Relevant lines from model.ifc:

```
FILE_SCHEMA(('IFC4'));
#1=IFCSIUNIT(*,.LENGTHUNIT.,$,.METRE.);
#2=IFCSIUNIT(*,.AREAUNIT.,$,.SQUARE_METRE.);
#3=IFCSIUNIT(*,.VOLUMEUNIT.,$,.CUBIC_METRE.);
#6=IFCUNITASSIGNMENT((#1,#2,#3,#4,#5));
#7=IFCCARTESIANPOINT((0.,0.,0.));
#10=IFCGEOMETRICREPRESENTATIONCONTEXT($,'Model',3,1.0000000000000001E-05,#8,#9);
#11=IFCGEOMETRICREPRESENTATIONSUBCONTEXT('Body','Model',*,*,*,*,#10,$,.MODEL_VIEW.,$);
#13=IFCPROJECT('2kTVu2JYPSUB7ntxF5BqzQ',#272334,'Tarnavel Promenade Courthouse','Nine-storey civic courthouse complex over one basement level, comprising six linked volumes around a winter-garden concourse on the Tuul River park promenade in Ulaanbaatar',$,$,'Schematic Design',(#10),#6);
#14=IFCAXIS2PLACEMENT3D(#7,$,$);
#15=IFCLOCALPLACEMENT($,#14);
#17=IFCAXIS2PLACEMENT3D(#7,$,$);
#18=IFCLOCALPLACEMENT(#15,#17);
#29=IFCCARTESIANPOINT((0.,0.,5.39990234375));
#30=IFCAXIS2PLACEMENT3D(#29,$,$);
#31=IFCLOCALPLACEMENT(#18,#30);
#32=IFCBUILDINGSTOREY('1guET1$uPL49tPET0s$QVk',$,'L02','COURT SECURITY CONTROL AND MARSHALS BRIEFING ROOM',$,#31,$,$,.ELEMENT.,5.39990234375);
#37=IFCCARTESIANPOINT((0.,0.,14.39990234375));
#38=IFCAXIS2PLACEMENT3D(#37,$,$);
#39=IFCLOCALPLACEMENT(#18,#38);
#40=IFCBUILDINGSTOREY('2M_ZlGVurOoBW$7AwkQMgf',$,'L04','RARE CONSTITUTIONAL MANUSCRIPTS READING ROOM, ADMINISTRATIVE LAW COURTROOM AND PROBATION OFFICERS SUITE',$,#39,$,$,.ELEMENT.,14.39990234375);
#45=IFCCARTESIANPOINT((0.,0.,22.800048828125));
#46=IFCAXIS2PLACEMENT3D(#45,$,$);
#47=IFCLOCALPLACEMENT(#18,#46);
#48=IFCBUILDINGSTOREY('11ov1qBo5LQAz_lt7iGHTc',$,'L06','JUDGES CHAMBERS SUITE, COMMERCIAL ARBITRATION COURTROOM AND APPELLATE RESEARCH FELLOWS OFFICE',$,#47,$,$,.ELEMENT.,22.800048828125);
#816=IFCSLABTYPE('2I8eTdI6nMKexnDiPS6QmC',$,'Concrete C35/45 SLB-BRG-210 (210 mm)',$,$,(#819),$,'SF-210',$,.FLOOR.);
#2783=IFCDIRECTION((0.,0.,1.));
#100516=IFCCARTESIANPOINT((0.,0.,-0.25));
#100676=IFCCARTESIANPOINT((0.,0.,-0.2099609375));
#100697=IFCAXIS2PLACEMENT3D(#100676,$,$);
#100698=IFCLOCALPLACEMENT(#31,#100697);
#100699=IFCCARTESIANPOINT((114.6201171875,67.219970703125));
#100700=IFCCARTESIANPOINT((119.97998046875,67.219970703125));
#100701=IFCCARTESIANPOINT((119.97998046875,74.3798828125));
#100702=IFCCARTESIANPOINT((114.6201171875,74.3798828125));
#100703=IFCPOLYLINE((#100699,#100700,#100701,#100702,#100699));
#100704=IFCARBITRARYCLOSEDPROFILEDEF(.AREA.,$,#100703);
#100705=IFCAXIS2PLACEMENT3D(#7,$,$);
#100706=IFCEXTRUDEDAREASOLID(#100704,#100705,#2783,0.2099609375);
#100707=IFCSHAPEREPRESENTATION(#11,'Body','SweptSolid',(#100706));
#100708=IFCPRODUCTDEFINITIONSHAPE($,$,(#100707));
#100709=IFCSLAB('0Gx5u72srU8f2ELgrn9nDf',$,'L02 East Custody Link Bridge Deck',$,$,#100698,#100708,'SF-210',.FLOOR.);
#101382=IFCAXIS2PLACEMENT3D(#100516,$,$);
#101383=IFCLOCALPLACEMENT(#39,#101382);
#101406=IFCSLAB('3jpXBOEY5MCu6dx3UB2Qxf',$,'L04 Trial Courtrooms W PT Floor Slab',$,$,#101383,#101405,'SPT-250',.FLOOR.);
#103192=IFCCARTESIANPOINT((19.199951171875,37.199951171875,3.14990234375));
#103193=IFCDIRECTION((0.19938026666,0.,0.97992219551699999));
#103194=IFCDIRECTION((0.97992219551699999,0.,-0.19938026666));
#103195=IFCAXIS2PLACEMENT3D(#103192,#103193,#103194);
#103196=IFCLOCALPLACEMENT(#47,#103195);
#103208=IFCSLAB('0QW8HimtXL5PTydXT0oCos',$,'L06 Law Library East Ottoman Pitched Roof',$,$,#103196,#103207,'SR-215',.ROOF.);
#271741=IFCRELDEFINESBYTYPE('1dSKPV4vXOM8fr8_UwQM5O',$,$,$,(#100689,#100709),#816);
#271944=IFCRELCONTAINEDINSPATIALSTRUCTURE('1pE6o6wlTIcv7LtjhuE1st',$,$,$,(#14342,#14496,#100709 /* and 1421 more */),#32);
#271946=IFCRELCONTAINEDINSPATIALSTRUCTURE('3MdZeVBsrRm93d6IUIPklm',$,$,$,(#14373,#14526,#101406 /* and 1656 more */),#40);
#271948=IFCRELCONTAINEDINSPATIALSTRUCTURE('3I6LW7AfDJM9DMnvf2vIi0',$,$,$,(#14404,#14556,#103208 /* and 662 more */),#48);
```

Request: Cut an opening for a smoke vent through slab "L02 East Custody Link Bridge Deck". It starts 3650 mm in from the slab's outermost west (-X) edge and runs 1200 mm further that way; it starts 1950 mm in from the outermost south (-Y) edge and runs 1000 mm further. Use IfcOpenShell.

```python
import numpy as np
import ifcopenshell
import ifcopenshell.api.feature
import ifcopenshell.api.geometry
import ifcopenshell.api.root
import ifcopenshell.geom
import ifcopenshell.util.placement
import ifcopenshell.util.representation
import ifcopenshell.util.shape
import ifcopenshell.util.unit

model = ifcopenshell.open("model.ifc")
unit_scale = ifcopenshell.util.unit.calculate_unit_scale(model)
settings = ifcopenshell.geom.settings()


def volume(element):
    """Net volume in cubic metres, openings subtracted."""
    shape = ifcopenshell.geom.create_shape(settings, element)
    return ifcopenshell.util.shape.get_volume(shape.geometry)


slab = model.by_guid("0Gx5u72srU8f2ELgrn9nDf")
before = volume(slab)

# Extent in the slab's own axes, in metres. The edges named are its -X and -Y sides.
slab_shape = ifcopenshell.geom.create_shape(settings, slab)
vertices = ifcopenshell.util.shape.get_vertices(slab_shape.geometry)
x_min, y_min, bottom = vertices.min(axis=0)
top = vertices[:, 2].max()

opening = ifcopenshell.api.root.create_entity(model, ifc_class="IfcOpeningElement", name="Smoke vent opening", predefined_type="OPENING")
context = ifcopenshell.util.representation.get_context(model, "Model", "Body", "MODEL_VIEW")
width, depth = 1.2, 1
outline = [(0.0, 0.0), (width, 0.0), (width, depth), (0.0, depth), (0.0, 0.0)]
# Overshoot both faces by 50 mm so the cut is clean.
shape = ifcopenshell.api.geometry.add_slab_representation(
    model, context=context, depth=top - bottom + 0.1, polyline=outline
)
ifcopenshell.api.geometry.assign_representation(model, product=opening, representation=shape)

matrix = ifcopenshell.util.placement.get_local_placement(slab.ObjectPlacement)
matrix[:, 3] = matrix @ np.append(np.array([x_min + 3.65, y_min + 1.95, bottom - 0.05]) / unit_scale, 1.0)
ifcopenshell.api.geometry.edit_object_placement(model, product=opening, matrix=matrix, is_si=False)
ifcopenshell.api.feature.add_feature(model, feature=opening, element=slab)

after = volume(slab)

print(f"slab volume {before:.3f} -> {after:.3f} m3")

model.write("model_rev.ifc")
```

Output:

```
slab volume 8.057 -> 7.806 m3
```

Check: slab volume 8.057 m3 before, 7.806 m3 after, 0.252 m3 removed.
